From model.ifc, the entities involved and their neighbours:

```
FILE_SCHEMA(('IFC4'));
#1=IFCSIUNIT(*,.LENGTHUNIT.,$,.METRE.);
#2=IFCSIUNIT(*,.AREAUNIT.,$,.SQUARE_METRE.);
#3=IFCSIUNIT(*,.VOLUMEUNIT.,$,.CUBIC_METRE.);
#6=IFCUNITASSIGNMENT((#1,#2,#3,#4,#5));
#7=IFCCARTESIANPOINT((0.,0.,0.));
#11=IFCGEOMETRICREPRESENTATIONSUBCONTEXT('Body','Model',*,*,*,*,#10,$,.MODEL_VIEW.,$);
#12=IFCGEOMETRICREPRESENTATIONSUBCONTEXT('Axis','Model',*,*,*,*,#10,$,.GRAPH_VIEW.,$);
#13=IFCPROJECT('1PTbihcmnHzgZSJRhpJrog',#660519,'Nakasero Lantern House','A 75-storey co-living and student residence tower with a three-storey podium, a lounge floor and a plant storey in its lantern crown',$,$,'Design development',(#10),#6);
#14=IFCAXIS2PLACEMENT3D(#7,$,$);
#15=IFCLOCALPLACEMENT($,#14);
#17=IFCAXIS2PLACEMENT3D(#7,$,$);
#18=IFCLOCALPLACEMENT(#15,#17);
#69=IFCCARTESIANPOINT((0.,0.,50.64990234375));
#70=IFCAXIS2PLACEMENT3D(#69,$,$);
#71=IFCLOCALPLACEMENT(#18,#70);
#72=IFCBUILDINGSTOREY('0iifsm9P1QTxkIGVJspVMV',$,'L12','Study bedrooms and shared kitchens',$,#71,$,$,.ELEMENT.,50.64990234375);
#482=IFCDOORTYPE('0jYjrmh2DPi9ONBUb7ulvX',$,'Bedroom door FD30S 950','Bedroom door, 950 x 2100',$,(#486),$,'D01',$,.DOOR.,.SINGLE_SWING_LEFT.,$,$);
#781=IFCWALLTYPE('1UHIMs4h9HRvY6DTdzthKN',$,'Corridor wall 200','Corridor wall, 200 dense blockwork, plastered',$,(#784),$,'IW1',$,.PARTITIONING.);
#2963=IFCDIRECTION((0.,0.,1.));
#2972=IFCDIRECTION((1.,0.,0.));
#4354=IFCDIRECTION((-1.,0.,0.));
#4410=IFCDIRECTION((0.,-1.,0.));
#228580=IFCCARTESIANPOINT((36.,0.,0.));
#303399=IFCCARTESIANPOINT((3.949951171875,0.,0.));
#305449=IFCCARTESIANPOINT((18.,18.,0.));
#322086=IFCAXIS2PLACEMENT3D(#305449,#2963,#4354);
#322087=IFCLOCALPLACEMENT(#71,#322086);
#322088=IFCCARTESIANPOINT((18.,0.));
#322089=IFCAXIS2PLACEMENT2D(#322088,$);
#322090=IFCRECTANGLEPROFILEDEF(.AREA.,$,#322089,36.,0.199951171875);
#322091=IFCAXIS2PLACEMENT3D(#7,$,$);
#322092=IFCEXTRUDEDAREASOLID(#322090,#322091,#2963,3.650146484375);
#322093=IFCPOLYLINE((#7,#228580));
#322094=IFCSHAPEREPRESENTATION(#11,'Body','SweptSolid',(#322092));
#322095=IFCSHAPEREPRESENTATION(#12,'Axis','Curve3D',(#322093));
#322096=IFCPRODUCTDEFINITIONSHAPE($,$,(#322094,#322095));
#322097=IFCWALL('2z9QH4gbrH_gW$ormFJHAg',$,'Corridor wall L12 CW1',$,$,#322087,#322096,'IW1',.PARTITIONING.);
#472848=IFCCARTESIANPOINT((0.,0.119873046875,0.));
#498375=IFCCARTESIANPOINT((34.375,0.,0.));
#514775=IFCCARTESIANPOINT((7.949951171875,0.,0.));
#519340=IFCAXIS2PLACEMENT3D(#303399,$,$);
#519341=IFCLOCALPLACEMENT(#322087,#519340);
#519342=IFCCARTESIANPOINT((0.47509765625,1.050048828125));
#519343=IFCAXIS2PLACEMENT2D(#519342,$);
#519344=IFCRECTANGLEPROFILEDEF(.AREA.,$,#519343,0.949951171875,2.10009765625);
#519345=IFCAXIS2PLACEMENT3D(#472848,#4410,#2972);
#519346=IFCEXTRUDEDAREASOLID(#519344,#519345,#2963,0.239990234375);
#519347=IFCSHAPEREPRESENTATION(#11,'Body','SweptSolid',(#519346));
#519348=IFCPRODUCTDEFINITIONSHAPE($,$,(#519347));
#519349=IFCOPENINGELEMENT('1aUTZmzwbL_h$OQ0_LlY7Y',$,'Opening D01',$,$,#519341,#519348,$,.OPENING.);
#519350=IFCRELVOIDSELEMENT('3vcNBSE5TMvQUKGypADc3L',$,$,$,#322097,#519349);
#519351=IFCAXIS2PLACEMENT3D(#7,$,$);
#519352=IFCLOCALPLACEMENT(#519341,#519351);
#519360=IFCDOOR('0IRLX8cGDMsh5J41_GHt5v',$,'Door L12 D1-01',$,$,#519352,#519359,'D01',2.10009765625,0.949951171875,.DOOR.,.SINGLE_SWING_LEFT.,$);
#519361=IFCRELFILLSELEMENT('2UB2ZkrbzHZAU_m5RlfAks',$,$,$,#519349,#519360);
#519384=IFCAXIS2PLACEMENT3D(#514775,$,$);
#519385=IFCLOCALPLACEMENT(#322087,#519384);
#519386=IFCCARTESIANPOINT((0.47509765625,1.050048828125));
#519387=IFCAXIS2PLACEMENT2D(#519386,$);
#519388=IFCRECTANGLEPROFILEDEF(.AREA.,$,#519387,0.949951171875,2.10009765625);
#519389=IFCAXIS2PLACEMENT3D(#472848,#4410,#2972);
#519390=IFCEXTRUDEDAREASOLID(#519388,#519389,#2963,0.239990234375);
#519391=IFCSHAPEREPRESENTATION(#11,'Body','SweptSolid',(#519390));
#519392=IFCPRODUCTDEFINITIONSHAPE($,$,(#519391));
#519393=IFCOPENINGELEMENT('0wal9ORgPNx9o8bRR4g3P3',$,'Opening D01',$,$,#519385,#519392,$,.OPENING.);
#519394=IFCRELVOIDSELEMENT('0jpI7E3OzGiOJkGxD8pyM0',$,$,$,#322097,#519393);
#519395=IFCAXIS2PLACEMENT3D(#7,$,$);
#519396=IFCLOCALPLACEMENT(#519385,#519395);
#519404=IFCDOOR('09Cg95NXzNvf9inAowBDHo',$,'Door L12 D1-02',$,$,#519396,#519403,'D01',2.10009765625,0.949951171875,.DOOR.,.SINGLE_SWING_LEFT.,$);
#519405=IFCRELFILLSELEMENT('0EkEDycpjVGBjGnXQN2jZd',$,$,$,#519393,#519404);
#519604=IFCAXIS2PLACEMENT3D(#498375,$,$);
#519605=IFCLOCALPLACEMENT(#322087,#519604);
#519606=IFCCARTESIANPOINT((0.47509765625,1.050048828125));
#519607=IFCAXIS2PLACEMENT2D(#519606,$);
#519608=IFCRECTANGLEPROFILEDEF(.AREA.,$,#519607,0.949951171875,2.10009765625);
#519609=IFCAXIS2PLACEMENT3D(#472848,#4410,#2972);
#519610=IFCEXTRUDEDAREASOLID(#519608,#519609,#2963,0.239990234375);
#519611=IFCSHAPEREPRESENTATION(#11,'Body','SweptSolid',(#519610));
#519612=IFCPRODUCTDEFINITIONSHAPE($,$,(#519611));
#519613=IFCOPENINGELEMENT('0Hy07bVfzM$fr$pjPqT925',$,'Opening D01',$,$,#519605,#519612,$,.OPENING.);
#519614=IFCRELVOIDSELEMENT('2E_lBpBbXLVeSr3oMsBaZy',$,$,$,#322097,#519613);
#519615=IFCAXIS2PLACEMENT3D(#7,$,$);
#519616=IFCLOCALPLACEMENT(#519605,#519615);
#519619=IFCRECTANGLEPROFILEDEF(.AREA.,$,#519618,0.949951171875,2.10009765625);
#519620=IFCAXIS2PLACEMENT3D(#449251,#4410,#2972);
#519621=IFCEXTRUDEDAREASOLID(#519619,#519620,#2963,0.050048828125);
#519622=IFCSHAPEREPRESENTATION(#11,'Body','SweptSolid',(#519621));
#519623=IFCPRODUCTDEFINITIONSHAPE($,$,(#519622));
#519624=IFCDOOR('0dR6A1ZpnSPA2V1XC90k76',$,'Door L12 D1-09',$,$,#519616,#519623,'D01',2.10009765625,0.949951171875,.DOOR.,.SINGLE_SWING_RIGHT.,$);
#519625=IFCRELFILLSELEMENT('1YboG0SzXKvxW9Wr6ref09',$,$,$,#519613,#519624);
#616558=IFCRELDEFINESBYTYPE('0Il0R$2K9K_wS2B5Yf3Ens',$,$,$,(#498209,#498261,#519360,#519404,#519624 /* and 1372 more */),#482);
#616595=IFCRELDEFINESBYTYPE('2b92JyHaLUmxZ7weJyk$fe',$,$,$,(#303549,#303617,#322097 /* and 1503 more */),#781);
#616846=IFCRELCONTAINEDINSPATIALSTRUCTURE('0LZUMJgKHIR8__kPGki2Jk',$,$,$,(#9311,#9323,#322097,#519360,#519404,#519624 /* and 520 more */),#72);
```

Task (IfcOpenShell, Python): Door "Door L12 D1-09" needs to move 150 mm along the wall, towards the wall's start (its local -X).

```python
import ifcopenshell
import ifcopenshell.api.geometry
import ifcopenshell.util.placement

model = ifcopenshell.open("model.ifc")

door = model.by_guid("0dR6A1ZpnSPA2V1XC90k76")
opening = door.FillsVoids[0].RelatingOpeningElement
wall = opening.VoidsElements[0].RelatingBuildingElement

wall_matrix = ifcopenshell.util.placement.get_local_placement(wall.ObjectPlacement)
shift = wall_matrix[:3, 0] * -0.15
before = ifcopenshell.util.placement.get_local_placement(door.ObjectPlacement)[:3, 3].copy()

# The door is placed relative to its opening, so it follows when the opening moves.
matrix = ifcopenshell.util.placement.get_local_placement(opening.ObjectPlacement)
matrix[:3, 3] += shift
ifcopenshell.api.geometry.edit_object_placement(
    model, product=opening, matrix=matrix, is_si=False, should_transform_children=True
)

after = ifcopenshell.util.placement.get_local_placement(door.ObjectPlacement)[:3, 3]
print("door moved by", (after - before).round(3) + 0.0)

model.write("model_updated.ifc")
```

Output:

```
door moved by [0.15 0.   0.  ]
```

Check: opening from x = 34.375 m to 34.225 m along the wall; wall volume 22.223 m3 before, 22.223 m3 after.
